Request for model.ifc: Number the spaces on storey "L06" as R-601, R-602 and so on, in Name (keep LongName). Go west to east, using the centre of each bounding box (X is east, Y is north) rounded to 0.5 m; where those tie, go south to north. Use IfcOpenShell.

First a look at what the model holds.

```python
import ifcopenshell
import ifcopenshell.util.element
import ifcopenshell.util.placement

model = ifcopenshell.open("model.ifc")
print(model.schema)
storey = next(s for s in model.by_type("IfcBuildingStorey") if s.Name == "L06")
spaces = [e for e in ifcopenshell.util.element.get_decomposition(storey) if e.is_a("IfcSpace")]
for e in sorted(spaces, key=lambda e: e.id()):
    origin = ifcopenshell.util.placement.get_local_placement(e.ObjectPlacement)[:3, 3]
    print(e.id(), e.Name, e.LongName, origin.round(2) + 0.0, sep=" | ")
```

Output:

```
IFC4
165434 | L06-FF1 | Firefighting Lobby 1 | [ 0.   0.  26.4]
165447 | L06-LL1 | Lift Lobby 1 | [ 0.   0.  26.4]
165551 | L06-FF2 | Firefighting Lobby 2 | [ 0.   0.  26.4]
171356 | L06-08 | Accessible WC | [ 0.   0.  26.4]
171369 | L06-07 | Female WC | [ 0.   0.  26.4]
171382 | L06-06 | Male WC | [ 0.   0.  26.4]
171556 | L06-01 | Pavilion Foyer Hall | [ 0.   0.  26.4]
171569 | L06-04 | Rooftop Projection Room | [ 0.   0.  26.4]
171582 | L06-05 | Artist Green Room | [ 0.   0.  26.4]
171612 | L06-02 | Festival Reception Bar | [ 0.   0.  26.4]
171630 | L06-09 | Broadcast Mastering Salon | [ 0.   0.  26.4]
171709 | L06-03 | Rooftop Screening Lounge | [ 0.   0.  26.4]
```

```python
import ifcopenshell
import ifcopenshell.geom
import ifcopenshell.util.element
import ifcopenshell.util.shape

model = ifcopenshell.open("model.ifc")
settings = ifcopenshell.geom.settings()
settings.set("use-world-coords", True)


def centre(element):
    shape = ifcopenshell.geom.create_shape(settings, element)
    return ifcopenshell.util.shape.get_bbox_centroid(shape.geometry)


storey = next(s for s in model.by_type("IfcBuildingStorey") if s.Name == "L06")
spaces = [e for e in ifcopenshell.util.element.get_decomposition(storey) if e.is_a("IfcSpace")]

# Insertion points can sit at a corner or the storey origin, so sort by the geometry (in metres).
centres = {e: centre(e) for e in spaces}
spaces.sort(key=lambda e: (round(centres[e][0] / 0.5), centres[e][1]))

for i, e in enumerate(spaces, start=1):
    number = f"R-6{i:02d}"
    e.Name = number
    print(e.id(), number)

model.write("model_v2.ifc")
```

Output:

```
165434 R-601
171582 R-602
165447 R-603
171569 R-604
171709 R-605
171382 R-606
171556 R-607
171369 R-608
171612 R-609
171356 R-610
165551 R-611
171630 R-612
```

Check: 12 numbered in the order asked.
